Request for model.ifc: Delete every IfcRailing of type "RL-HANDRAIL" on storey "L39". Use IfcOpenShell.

First a look at what the model holds.

```python
import ifcopenshell
import ifcopenshell.util.element

model = ifcopenshell.open("model.ifc")
print(model.schema)
storey = next(s for s in model.by_type("IfcBuildingStorey") if s.Name == "L39")
railings = [e for e in ifcopenshell.util.element.get_decomposition(storey) if e.is_a("IfcRailing")]
seen = {}
for e in railings:
    element_type = ifcopenshell.util.element.get_type(e)
    name = element_type.Name if element_type not in (None, e) else None
    seen[name] = seen.get(name, 0) + 1
for name, count in sorted(seen.items(), key=str):
    print(count, "x", name)
```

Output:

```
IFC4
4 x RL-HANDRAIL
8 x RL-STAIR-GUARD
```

```python
import ifcopenshell
import ifcopenshell.api.root
import ifcopenshell.util.element

model = ifcopenshell.open("model.ifc")

storey = next(s for s in model.by_type("IfcBuildingStorey") if s.Name == "L39")
railings = [e for e in ifcopenshell.util.element.get_decomposition(storey) if e.is_a("IfcRailing")]
targets = [e for e in railings if (t := ifcopenshell.util.element.get_type(e)) not in (None, e) and t.Name == "RL-HANDRAIL"]

for e in targets:
    ifcopenshell.api.root.remove_product(model, product=e)
print(len(targets), "removed")

model.write("model_rev.ifc")
```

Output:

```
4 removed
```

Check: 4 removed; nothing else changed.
